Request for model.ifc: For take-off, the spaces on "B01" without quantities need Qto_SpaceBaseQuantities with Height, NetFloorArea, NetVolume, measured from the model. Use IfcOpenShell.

First a look at what the model holds.

```python
import ifcopenshell
import ifcopenshell.util.element
import ifcopenshell.util.unit

model = ifcopenshell.open("model.ifc")
print(model.schema)
for unit_type in ("LENGTHUNIT", "AREAUNIT", "VOLUMEUNIT"):
    print(unit_type, ifcopenshell.util.unit.calculate_unit_scale(model, unit_type))
storey = next(s for s in model.by_type("IfcBuildingStorey") if s.Name == "B01")
spaces = [e for e in ifcopenshell.util.element.get_decomposition(storey) if e.is_a("IfcSpace")]
for e in sorted(spaces, key=lambda e: e.id()):
    print(e.id(), e.is_a(), e.Name, list(ifcopenshell.util.element.get_psets(e, qtos_only=True)), sep=" | ")
```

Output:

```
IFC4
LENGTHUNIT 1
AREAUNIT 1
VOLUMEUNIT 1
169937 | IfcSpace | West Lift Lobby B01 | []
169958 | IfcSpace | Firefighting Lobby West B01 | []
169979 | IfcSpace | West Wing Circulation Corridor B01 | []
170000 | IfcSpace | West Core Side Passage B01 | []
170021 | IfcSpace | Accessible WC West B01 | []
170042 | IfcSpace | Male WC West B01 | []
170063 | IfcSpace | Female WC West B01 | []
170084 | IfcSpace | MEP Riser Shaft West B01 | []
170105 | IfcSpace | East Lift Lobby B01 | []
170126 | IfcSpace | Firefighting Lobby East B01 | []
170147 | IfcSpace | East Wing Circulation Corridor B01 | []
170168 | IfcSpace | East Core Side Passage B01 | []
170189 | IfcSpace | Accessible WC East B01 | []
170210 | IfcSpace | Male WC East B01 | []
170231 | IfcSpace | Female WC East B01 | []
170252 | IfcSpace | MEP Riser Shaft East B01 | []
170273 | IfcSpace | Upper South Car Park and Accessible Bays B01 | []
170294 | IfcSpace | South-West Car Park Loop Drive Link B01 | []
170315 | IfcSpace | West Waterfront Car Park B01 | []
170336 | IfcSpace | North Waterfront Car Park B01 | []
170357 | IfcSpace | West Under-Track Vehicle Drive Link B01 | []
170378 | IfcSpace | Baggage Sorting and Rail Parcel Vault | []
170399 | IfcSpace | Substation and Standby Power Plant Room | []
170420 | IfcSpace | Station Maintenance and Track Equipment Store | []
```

```python
import ifcopenshell
import ifcopenshell.api.pset
import ifcopenshell.geom
import ifcopenshell.util.element
import ifcopenshell.util.shape
import ifcopenshell.util.unit

model = ifcopenshell.open("model.ifc")
unit_scale = ifcopenshell.util.unit.calculate_unit_scale(model)
area_scale = ifcopenshell.util.unit.calculate_unit_scale(model, "AREAUNIT")
volume_scale = ifcopenshell.util.unit.calculate_unit_scale(model, "VOLUMEUNIT")
settings = ifcopenshell.geom.settings()

storey = next(s for s in model.by_type("IfcBuildingStorey") if s.Name == "B01")
spaces = [e for e in ifcopenshell.util.element.get_decomposition(storey) if e.is_a("IfcSpace")]

for e in sorted(spaces, key=lambda e: e.id()):
    if ifcopenshell.util.element.get_psets(e, qtos_only=True, should_inherit=False):
        continue
    # Geometry comes back in metres, in the element's own axes.
    shape = ifcopenshell.geom.create_shape(settings, e)
    values = {
        "Height": ifcopenshell.util.shape.get_z(shape.geometry) / unit_scale,
        "NetFloorArea": ifcopenshell.util.shape.get_footprint_area(shape.geometry) / area_scale,
        "NetVolume": ifcopenshell.util.shape.get_volume(shape.geometry) / volume_scale,
    }
    qto = ifcopenshell.api.pset.add_qto(model, product=e, name="Qto_SpaceBaseQuantities")
    ifcopenshell.api.pset.edit_qto(model, qto=qto, properties=values)
    print(e.id(), {k: round(v, 3) for k, v in values.items()})

model.write("model_rev.ifc")
```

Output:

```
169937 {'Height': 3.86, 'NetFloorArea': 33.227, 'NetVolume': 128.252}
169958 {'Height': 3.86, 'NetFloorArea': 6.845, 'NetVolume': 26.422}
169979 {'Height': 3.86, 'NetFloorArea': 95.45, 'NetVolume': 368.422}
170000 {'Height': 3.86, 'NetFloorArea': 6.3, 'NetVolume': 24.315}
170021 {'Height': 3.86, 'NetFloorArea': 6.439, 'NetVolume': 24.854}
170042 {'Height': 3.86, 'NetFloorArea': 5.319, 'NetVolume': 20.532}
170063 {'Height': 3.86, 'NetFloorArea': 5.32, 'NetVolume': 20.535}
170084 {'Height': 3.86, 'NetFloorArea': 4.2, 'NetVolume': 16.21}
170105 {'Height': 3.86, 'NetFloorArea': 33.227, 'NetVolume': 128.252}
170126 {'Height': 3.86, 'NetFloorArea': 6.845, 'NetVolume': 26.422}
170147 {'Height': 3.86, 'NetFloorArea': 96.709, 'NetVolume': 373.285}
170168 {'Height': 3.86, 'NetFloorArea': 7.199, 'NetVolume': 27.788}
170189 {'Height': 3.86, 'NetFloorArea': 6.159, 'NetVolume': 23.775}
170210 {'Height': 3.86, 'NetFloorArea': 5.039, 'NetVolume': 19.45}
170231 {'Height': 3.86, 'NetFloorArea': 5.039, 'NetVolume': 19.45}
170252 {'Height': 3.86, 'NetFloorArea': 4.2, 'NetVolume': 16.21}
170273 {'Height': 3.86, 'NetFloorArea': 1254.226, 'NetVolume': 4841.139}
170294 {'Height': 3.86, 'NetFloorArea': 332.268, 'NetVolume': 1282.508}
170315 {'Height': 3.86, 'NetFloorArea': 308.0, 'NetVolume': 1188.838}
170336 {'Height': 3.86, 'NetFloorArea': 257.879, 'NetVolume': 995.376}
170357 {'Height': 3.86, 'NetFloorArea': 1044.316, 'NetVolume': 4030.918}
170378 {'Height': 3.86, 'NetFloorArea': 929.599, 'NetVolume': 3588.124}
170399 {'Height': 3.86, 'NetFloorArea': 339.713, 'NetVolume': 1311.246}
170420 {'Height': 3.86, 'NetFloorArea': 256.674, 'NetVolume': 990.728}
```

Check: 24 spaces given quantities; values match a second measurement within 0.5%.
